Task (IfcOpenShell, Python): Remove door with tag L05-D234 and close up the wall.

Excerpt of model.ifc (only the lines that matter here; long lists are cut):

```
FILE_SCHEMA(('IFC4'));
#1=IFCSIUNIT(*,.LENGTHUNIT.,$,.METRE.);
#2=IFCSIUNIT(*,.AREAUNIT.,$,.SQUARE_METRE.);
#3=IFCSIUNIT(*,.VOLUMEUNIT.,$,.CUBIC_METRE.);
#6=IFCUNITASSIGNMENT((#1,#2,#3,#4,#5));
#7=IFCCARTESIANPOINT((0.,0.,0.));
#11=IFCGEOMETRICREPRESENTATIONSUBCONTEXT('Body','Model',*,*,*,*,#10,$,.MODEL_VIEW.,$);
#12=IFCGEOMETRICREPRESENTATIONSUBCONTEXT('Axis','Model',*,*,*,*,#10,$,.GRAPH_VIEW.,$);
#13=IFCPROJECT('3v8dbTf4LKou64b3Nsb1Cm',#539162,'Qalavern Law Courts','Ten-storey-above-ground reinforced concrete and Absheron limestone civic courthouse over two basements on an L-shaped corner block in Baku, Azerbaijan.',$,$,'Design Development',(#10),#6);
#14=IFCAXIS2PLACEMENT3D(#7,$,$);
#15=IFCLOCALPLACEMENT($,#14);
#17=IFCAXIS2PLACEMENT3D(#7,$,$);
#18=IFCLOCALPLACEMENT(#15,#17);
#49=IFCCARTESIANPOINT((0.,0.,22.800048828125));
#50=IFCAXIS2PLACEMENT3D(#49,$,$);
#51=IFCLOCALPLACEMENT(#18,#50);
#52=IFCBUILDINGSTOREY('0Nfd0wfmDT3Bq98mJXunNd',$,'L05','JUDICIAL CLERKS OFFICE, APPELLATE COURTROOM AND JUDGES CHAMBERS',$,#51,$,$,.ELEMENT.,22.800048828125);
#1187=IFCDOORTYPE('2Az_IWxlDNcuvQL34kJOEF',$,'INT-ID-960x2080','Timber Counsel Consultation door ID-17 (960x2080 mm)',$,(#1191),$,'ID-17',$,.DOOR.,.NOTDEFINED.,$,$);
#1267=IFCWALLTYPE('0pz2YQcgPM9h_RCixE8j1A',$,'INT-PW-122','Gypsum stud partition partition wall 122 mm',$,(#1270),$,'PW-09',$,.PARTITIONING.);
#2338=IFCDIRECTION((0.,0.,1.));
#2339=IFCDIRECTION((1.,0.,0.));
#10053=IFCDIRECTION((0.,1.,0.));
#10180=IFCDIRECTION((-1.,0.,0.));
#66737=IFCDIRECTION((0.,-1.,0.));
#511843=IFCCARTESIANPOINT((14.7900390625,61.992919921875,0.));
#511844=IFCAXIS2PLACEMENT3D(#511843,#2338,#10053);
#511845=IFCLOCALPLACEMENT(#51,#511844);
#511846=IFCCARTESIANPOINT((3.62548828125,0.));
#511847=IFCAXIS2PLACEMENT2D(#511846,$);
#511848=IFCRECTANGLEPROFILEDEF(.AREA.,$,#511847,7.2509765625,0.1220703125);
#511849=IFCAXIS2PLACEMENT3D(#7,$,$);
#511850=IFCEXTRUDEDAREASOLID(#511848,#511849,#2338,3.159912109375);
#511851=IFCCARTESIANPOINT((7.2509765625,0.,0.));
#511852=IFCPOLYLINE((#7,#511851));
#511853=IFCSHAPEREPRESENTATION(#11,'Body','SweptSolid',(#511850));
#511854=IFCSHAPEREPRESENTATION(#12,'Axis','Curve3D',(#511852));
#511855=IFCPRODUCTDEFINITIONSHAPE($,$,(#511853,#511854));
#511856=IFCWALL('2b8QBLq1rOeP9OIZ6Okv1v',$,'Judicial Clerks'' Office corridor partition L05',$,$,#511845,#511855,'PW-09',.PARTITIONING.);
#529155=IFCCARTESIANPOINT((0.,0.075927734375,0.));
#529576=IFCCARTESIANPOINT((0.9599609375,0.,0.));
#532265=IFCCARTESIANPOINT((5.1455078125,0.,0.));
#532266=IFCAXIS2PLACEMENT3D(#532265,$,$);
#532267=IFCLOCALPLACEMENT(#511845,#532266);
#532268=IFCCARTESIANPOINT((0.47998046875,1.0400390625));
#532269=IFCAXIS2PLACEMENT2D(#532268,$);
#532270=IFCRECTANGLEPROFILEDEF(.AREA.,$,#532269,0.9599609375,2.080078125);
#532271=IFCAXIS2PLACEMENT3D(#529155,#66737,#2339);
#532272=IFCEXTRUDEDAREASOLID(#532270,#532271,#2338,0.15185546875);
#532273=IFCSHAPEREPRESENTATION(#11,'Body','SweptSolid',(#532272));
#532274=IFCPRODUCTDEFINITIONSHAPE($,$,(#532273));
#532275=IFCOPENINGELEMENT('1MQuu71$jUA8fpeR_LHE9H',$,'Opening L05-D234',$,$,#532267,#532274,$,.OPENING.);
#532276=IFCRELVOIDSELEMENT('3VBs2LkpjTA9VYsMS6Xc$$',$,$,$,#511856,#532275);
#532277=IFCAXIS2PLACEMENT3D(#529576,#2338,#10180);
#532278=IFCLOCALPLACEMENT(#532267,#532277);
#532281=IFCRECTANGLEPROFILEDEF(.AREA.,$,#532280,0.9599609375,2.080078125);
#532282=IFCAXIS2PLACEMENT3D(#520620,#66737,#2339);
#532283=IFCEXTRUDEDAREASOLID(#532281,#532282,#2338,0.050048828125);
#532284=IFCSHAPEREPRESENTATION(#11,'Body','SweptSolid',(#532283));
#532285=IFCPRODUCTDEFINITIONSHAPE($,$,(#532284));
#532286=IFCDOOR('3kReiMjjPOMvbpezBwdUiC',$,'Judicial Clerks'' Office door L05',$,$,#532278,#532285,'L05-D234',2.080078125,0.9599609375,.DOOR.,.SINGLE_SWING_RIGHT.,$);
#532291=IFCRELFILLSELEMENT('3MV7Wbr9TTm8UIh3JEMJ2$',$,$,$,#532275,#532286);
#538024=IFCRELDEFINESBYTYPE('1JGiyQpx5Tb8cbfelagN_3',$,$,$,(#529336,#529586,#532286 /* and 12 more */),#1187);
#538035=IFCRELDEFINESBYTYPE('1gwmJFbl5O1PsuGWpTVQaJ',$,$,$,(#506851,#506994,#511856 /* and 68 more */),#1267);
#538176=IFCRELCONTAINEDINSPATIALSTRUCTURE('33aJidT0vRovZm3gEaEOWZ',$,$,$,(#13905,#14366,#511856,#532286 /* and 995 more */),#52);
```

```python
import ifcopenshell
import ifcopenshell.api.feature
import ifcopenshell.api.root
import ifcopenshell.geom
import ifcopenshell.util.shape

model = ifcopenshell.open("model.ifc")
settings = ifcopenshell.geom.settings()


def volume(element):
    """Net volume in cubic metres, openings subtracted."""
    shape = ifcopenshell.geom.create_shape(settings, element)
    return ifcopenshell.util.shape.get_volume(shape.geometry)


door = model.by_guid("3kReiMjjPOMvbpezBwdUiC")
opening = door.FillsVoids[0].RelatingOpeningElement
wall = opening.VoidsElements[0].RelatingBuildingElement
before = volume(wall)

ifcopenshell.api.root.remove_product(model, product=door)
ifcopenshell.api.feature.remove_feature(model, feature=opening)

after = volume(wall)

print(f"wall volume {before:.3f} -> {after:.3f} m3")

model.write("model_rev.ifc")
```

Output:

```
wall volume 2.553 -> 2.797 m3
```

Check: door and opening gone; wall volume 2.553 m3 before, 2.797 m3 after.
